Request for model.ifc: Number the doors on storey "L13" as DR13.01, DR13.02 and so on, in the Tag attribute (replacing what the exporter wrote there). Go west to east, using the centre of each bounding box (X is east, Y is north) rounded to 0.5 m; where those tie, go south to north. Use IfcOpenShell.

First a look at what the model holds.

```python
import ifcopenshell
import ifcopenshell.util.element
import ifcopenshell.util.placement

model = ifcopenshell.open("model.ifc")
print(model.schema)
storey = next(s for s in model.by_type("IfcBuildingStorey") if s.Name == "L13")
doors = [e for e in ifcopenshell.util.element.get_decomposition(storey) if e.is_a("IfcDoor")]
for e in sorted(doors, key=lambda e: e.id()):
    origin = ifcopenshell.util.placement.get_local_placement(e.ObjectPlacement)[:3, 3]
    print(e.id(), e.Tag, e.Name, origin.round(2) + 0.0, sep=" | ")
```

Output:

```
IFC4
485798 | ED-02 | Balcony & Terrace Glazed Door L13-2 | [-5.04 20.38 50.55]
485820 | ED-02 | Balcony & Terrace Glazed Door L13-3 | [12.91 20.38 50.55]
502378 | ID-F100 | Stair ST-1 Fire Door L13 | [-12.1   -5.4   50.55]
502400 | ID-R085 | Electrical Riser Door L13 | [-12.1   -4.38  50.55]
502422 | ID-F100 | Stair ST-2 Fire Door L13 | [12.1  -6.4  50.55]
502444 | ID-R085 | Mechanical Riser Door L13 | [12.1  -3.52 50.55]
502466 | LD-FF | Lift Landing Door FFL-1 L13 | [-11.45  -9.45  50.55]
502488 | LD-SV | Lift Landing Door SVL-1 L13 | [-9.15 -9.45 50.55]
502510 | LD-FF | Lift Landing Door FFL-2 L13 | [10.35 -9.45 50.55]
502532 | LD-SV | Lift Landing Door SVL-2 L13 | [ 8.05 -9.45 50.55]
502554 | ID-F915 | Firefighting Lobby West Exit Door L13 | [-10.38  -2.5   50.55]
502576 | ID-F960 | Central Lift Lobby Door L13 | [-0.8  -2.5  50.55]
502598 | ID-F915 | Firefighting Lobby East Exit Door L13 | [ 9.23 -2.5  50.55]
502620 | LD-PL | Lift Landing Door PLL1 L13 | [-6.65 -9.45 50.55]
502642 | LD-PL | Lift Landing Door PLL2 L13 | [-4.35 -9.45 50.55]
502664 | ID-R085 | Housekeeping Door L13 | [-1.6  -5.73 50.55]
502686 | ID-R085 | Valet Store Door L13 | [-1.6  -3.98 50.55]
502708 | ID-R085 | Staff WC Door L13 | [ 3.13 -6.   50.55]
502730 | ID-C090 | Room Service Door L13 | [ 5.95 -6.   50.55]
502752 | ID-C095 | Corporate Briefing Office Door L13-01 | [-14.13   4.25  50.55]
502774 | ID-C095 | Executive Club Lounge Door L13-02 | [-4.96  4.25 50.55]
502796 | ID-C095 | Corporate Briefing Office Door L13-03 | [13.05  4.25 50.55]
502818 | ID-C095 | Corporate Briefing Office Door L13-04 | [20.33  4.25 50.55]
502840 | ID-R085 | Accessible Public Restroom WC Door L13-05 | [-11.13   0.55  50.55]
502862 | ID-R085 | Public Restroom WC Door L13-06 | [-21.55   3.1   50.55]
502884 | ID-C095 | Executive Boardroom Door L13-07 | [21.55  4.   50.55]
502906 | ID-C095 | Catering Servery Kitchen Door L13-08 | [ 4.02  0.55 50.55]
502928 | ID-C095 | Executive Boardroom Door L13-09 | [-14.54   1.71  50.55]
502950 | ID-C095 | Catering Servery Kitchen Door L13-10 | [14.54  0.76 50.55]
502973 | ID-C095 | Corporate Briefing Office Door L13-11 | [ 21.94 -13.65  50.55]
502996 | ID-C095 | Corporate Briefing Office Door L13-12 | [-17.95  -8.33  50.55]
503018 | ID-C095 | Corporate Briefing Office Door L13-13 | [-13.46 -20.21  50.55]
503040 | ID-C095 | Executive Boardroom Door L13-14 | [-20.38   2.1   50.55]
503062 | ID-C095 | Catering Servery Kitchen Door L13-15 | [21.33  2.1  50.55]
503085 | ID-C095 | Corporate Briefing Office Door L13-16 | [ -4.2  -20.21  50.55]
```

```python
import ifcopenshell
import ifcopenshell.geom
import ifcopenshell.util.element
import ifcopenshell.util.shape

model = ifcopenshell.open("model.ifc")
settings = ifcopenshell.geom.settings()
settings.set("use-world-coords", True)


def centre(element):
    shape = ifcopenshell.geom.create_shape(settings, element)
    return ifcopenshell.util.shape.get_bbox_centroid(shape.geometry)


storey = next(s for s in model.by_type("IfcBuildingStorey") if s.Name == "L13")
doors = [e for e in ifcopenshell.util.element.get_decomposition(storey) if e.is_a("IfcDoor")]

# Insertion points can sit at a corner or the storey origin, so sort by the geometry (in metres).
centres = {e: centre(e) for e in doors}
doors.sort(key=lambda e: (round(centres[e][0] / 0.5), centres[e][1]))

for i, e in enumerate(doors, start=1):
    number = f"DR13.{i:02d}"
    e.Tag = number
    print(e.id(), number)

model.write("model_rev.ifc")
```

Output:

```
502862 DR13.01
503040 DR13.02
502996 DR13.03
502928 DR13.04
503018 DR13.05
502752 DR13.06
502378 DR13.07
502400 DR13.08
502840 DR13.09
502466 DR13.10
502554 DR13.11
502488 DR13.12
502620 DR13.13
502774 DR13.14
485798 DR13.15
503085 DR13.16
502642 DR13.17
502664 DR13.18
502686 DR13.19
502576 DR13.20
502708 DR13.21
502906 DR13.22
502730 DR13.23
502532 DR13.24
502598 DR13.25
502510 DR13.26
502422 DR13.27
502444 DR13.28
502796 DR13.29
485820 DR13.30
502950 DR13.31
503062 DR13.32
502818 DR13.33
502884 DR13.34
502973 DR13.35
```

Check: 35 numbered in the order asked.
